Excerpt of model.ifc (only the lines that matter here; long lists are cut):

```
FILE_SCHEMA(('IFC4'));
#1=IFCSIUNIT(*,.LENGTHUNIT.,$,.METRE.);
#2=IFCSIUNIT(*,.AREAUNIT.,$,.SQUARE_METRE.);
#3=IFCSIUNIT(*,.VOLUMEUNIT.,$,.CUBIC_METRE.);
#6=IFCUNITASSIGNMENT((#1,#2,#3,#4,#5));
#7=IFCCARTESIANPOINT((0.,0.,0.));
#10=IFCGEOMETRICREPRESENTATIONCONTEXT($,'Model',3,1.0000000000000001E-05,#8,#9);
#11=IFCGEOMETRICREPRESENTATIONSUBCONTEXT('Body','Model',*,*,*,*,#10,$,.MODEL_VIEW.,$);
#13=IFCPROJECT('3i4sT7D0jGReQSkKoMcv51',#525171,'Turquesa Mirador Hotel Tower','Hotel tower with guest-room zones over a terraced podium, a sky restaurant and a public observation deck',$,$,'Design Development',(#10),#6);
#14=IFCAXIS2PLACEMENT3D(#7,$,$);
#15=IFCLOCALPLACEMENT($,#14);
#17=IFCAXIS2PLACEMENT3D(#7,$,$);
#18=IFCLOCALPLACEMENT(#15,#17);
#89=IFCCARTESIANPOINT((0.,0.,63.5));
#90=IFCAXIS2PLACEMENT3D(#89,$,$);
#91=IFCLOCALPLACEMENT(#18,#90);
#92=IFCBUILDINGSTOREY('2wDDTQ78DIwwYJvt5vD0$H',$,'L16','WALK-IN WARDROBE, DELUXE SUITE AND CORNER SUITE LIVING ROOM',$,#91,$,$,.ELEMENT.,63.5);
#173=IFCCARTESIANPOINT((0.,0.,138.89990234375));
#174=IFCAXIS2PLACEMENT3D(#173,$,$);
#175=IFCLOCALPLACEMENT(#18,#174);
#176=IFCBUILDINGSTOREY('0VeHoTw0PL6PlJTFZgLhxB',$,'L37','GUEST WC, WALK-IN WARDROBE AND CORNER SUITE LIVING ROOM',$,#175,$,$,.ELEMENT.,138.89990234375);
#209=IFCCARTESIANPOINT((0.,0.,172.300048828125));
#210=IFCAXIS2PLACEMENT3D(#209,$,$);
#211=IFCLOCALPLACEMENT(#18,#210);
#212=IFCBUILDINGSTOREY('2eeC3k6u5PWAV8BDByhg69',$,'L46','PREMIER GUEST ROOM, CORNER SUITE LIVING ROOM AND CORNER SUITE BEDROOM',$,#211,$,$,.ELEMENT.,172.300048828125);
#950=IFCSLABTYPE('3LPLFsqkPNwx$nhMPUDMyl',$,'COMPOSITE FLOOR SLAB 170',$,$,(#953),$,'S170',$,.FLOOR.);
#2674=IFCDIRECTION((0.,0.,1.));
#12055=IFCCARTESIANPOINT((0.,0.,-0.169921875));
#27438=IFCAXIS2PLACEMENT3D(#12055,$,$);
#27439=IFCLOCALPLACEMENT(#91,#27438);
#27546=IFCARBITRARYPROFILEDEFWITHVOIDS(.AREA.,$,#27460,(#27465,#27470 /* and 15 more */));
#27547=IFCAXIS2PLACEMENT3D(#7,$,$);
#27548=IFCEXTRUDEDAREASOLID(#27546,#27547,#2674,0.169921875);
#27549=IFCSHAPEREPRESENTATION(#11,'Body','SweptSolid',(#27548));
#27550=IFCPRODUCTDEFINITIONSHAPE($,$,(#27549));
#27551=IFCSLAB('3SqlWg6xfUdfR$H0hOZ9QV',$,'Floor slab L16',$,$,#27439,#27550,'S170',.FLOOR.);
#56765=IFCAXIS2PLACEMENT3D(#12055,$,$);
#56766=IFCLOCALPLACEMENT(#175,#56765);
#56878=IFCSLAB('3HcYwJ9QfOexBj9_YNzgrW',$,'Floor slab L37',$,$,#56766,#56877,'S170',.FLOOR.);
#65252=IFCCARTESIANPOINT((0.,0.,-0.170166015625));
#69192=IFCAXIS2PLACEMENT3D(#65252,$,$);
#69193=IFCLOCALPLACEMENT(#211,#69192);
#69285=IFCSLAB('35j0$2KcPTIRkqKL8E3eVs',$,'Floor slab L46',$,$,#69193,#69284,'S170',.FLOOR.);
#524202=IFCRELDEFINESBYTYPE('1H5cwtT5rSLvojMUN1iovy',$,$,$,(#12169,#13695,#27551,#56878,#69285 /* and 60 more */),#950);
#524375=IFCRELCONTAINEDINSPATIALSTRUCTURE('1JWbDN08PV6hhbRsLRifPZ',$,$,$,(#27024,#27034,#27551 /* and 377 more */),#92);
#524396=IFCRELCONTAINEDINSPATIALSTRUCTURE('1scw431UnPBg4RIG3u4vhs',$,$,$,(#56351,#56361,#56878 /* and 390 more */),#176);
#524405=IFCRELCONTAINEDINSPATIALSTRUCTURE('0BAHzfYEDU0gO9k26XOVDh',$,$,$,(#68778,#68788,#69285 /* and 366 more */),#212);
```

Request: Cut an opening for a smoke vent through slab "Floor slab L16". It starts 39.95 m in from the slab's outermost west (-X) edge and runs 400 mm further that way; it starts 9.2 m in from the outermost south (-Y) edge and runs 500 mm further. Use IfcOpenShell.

```python
import numpy as np
import ifcopenshell
import ifcopenshell.api.feature
import ifcopenshell.api.geometry
import ifcopenshell.api.root
import ifcopenshell.geom
import ifcopenshell.util.placement
import ifcopenshell.util.representation
import ifcopenshell.util.shape
import ifcopenshell.util.unit

model = ifcopenshell.open("model.ifc")
unit_scale = ifcopenshell.util.unit.calculate_unit_scale(model)
settings = ifcopenshell.geom.settings()


def volume(element):
    """Net volume in cubic metres, openings subtracted."""
    shape = ifcopenshell.geom.create_shape(settings, element)
    return ifcopenshell.util.shape.get_volume(shape.geometry)


slab = model.by_guid("3SqlWg6xfUdfR$H0hOZ9QV")
before = volume(slab)

# Extent in the slab's own axes, in metres. The edges named are its -X and -Y sides.
slab_shape = ifcopenshell.geom.create_shape(settings, slab)
vertices = ifcopenshell.util.shape.get_vertices(slab_shape.geometry)
x_min, y_min, bottom = vertices.min(axis=0)
top = vertices[:, 2].max()

opening = ifcopenshell.api.root.create_entity(model, ifc_class="IfcOpeningElement", name="Smoke vent opening", predefined_type="OPENING")
context = ifcopenshell.util.representation.get_context(model, "Model", "Body", "MODEL_VIEW")
width, depth = 0.4, 0.5
outline = [(0.0, 0.0), (width, 0.0), (width, depth), (0.0, depth), (0.0, 0.0)]
# Overshoot both faces by 50 mm so the cut is clean.
shape = ifcopenshell.api.geometry.add_slab_representation(
    model, context=context, depth=top - bottom + 0.1, polyline=outline
)
ifcopenshell.api.geometry.assign_representation(model, product=opening, representation=shape)

matrix = ifcopenshell.util.placement.get_local_placement(slab.ObjectPlacement)
matrix[:, 3] = matrix @ np.append(np.array([x_min + 39.95, y_min + 9.2, bottom - 0.05]) / unit_scale, 1.0)
ifcopenshell.api.geometry.edit_object_placement(model, product=opening, matrix=matrix, is_si=False)
ifcopenshell.api.feature.add_feature(model, feature=opening, element=slab)

after = volume(slab)

print(f"slab volume {before:.3f} -> {after:.3f} m3")

model.write("model_updated.ifc")
```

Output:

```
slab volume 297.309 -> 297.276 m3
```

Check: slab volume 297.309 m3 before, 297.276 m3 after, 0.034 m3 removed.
